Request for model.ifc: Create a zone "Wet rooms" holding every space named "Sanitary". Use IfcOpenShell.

First a look at what the model holds.

```python
import ifcopenshell

model = ifcopenshell.open("model.ifc")
print(model.schema)
seen = {}
for space in model.by_type("IfcSpace"):
    seen[space.LongName] = seen.get(space.LongName, 0) + 1
for name, count in sorted(seen.items(), key=str):
    print(count, "x", name)
print("zones:", [z.Name for z in model.by_type("IfcZone")][:20])
```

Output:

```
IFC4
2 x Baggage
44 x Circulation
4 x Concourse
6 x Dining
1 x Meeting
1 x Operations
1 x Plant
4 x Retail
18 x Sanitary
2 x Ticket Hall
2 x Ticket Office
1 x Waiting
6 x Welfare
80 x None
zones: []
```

```python
import ifcopenshell
import ifcopenshell.api.group
import ifcopenshell.api.root

model = ifcopenshell.open("model.ifc")

names = {"Sanitary"}
spaces = [s for s in model.by_type("IfcSpace") if s.LongName in names]

zone = ifcopenshell.api.root.create_entity(model, ifc_class="IfcZone", name="Wet rooms")
ifcopenshell.api.group.assign_group(model, products=spaces, group=zone)
print(len(spaces), "spaces in", zone.Name)

model.write("model-out.ifc")
```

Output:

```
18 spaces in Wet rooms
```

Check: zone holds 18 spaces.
